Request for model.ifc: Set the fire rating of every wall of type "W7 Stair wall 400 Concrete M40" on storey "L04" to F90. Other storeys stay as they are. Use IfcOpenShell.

First a look at what the model holds.

```python
import ifcopenshell
import ifcopenshell.util.element

model = ifcopenshell.open("model.ifc")
print(model.schema)
storey = next(s for s in model.by_type("IfcBuildingStorey") if s.Name == "L04")
walls = [e for e in ifcopenshell.util.element.get_decomposition(storey) if e.is_a("IfcWall")]
seen = {}
for e in walls:
    element_type = ifcopenshell.util.element.get_type(e)
    key = (element_type.Name if element_type != e and element_type else None, ifcopenshell.util.element.get_pset(e, "Pset_WallCommon", "FireRating"))
    seen[key] = seen.get(key, 0) + 1
for (name, value), count in sorted(seen.items(), key=str):
    print(count, "x", name, "|", value)
```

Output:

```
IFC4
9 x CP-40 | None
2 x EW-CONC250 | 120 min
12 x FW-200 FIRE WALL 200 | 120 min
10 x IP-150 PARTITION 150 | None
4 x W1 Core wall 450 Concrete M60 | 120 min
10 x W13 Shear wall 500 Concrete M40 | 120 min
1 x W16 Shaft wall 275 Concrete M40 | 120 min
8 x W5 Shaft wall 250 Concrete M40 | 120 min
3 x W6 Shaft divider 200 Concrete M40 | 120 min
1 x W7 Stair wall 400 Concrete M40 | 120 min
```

```python
import ifcopenshell
import ifcopenshell.api.pset
import ifcopenshell.util.element

model = ifcopenshell.open("model.ifc")

storey = next(s for s in model.by_type("IfcBuildingStorey") if s.Name == "L04")
walls = [e for e in ifcopenshell.util.element.get_decomposition(storey) if e.is_a("IfcWall")]

count = 0
for e in walls:
    element_type = ifcopenshell.util.element.get_type(e)
    if element_type in (None, e) or element_type.Name != "W7 Stair wall 400 Concrete M40":
        continue
    # add_pset returns the element's existing set when there is one.
    pset = ifcopenshell.api.pset.add_pset(model, product=e, name="Pset_WallCommon")
    ifcopenshell.api.pset.edit_pset(model, pset=pset, properties={"FireRating": "F90"})
    count += 1

print(count, "walls updated")

model.write("model_updated.ifc")
```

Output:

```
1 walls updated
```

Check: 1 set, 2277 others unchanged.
